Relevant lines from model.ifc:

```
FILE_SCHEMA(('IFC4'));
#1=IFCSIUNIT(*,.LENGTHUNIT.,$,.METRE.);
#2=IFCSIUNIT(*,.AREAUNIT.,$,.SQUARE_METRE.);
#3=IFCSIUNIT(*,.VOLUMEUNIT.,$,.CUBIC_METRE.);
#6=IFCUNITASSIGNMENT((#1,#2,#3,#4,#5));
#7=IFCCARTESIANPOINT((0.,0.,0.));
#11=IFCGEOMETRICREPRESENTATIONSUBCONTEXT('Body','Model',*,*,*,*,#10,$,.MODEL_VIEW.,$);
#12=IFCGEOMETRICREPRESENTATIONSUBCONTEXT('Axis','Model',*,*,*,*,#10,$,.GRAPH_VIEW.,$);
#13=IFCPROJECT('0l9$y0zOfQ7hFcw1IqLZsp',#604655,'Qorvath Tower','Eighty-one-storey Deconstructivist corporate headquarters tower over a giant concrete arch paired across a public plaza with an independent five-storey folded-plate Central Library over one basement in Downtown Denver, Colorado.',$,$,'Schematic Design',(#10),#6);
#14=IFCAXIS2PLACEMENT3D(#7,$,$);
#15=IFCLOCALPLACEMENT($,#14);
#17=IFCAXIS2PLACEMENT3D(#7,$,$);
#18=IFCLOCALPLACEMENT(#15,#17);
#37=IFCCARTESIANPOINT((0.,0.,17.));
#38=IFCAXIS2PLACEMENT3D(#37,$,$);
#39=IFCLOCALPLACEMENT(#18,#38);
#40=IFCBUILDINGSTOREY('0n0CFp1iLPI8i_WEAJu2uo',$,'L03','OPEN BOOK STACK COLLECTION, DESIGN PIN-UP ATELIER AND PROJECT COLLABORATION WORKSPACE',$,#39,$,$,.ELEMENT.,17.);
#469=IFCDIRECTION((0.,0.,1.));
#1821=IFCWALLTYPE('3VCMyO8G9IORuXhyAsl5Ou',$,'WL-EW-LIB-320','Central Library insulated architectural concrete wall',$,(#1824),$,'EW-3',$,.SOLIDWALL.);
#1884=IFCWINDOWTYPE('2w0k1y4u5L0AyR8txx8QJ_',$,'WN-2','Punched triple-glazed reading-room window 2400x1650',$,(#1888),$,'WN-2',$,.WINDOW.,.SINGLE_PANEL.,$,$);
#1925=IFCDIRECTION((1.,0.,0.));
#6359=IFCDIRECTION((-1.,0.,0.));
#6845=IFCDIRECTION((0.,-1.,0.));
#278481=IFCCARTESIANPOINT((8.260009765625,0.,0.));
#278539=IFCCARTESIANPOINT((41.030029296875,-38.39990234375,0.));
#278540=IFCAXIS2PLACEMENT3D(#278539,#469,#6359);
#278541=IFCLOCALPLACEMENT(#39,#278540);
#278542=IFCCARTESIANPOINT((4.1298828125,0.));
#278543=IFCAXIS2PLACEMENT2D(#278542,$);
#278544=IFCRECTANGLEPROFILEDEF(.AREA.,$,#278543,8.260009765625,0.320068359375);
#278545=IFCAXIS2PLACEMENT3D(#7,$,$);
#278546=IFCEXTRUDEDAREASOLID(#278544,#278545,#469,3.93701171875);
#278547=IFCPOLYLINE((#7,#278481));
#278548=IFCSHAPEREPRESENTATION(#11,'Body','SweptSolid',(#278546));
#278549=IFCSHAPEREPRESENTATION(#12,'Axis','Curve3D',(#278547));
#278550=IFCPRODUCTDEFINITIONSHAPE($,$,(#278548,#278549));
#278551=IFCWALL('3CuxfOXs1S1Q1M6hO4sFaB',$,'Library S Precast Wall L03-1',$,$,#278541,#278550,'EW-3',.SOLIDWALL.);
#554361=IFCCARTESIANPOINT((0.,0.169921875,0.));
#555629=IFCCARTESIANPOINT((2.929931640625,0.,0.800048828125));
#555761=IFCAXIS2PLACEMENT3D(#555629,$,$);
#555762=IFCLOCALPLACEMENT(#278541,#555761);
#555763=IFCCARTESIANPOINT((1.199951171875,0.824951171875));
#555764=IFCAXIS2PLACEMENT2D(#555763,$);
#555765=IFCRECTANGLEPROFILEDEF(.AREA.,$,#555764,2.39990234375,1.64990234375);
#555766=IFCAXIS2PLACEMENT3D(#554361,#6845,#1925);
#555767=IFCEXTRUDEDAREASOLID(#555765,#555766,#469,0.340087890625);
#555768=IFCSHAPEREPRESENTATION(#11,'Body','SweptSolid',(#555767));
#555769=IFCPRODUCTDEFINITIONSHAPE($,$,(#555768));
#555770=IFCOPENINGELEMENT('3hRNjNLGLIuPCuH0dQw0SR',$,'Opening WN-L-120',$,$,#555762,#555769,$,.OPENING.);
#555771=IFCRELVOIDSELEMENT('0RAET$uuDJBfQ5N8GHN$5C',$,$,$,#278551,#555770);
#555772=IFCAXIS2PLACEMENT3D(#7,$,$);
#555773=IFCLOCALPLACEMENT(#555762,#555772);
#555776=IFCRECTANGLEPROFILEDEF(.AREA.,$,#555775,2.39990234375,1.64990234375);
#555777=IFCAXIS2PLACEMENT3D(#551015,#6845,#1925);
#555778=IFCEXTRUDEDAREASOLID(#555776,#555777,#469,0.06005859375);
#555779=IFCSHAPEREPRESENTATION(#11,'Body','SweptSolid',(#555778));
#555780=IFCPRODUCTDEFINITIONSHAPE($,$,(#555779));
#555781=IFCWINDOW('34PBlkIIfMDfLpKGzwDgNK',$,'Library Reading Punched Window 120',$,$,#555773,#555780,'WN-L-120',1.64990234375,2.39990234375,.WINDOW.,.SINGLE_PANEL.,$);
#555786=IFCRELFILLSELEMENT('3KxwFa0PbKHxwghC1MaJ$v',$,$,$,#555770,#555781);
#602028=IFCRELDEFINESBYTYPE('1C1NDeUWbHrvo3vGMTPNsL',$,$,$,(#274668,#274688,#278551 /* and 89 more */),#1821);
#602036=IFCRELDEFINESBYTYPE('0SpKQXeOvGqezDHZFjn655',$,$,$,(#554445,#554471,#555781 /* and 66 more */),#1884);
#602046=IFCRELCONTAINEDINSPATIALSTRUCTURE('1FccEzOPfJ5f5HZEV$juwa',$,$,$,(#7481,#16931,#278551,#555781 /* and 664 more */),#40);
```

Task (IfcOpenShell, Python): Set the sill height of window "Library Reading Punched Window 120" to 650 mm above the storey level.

```python
import numpy as np
import ifcopenshell
import ifcopenshell.api.geometry
import ifcopenshell.geom
import ifcopenshell.util.element
import ifcopenshell.util.placement
import ifcopenshell.util.shape
import ifcopenshell.util.unit

model = ifcopenshell.open("model.ifc")
unit_scale = ifcopenshell.util.unit.calculate_unit_scale(model)

window = model.by_guid("34PBlkIIfMDfLpKGzwDgNK")
opening = window.FillsVoids[0].RelatingOpeningElement
storey = ifcopenshell.util.element.get_container(window, ifc_class="IfcBuildingStorey")
level = ifcopenshell.util.placement.get_local_placement(storey.ObjectPlacement)[2, 3]

# The opening's origin need not be at the sill, so measure its lowest point.
shape = ifcopenshell.geom.create_shape(ifcopenshell.geom.settings(), opening)
bottom = ifcopenshell.util.shape.get_shape_bottom_elevation(shape, shape.geometry) / unit_scale
dz = level + 0.65 - bottom

shift = np.array([0.0, 0.0, dz])
# The window is placed relative to its opening, so it follows when the opening moves.
matrix = ifcopenshell.util.placement.get_local_placement(opening.ObjectPlacement)
matrix[:3, 3] += shift
ifcopenshell.api.geometry.edit_object_placement(
    model, product=opening, matrix=matrix, is_si=False, should_transform_children=True
)

print(f"moved by {dz * unit_scale:+.3f} m")

model.write("model-out.ifc")
```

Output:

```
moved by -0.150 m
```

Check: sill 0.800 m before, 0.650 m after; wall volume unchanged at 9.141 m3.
